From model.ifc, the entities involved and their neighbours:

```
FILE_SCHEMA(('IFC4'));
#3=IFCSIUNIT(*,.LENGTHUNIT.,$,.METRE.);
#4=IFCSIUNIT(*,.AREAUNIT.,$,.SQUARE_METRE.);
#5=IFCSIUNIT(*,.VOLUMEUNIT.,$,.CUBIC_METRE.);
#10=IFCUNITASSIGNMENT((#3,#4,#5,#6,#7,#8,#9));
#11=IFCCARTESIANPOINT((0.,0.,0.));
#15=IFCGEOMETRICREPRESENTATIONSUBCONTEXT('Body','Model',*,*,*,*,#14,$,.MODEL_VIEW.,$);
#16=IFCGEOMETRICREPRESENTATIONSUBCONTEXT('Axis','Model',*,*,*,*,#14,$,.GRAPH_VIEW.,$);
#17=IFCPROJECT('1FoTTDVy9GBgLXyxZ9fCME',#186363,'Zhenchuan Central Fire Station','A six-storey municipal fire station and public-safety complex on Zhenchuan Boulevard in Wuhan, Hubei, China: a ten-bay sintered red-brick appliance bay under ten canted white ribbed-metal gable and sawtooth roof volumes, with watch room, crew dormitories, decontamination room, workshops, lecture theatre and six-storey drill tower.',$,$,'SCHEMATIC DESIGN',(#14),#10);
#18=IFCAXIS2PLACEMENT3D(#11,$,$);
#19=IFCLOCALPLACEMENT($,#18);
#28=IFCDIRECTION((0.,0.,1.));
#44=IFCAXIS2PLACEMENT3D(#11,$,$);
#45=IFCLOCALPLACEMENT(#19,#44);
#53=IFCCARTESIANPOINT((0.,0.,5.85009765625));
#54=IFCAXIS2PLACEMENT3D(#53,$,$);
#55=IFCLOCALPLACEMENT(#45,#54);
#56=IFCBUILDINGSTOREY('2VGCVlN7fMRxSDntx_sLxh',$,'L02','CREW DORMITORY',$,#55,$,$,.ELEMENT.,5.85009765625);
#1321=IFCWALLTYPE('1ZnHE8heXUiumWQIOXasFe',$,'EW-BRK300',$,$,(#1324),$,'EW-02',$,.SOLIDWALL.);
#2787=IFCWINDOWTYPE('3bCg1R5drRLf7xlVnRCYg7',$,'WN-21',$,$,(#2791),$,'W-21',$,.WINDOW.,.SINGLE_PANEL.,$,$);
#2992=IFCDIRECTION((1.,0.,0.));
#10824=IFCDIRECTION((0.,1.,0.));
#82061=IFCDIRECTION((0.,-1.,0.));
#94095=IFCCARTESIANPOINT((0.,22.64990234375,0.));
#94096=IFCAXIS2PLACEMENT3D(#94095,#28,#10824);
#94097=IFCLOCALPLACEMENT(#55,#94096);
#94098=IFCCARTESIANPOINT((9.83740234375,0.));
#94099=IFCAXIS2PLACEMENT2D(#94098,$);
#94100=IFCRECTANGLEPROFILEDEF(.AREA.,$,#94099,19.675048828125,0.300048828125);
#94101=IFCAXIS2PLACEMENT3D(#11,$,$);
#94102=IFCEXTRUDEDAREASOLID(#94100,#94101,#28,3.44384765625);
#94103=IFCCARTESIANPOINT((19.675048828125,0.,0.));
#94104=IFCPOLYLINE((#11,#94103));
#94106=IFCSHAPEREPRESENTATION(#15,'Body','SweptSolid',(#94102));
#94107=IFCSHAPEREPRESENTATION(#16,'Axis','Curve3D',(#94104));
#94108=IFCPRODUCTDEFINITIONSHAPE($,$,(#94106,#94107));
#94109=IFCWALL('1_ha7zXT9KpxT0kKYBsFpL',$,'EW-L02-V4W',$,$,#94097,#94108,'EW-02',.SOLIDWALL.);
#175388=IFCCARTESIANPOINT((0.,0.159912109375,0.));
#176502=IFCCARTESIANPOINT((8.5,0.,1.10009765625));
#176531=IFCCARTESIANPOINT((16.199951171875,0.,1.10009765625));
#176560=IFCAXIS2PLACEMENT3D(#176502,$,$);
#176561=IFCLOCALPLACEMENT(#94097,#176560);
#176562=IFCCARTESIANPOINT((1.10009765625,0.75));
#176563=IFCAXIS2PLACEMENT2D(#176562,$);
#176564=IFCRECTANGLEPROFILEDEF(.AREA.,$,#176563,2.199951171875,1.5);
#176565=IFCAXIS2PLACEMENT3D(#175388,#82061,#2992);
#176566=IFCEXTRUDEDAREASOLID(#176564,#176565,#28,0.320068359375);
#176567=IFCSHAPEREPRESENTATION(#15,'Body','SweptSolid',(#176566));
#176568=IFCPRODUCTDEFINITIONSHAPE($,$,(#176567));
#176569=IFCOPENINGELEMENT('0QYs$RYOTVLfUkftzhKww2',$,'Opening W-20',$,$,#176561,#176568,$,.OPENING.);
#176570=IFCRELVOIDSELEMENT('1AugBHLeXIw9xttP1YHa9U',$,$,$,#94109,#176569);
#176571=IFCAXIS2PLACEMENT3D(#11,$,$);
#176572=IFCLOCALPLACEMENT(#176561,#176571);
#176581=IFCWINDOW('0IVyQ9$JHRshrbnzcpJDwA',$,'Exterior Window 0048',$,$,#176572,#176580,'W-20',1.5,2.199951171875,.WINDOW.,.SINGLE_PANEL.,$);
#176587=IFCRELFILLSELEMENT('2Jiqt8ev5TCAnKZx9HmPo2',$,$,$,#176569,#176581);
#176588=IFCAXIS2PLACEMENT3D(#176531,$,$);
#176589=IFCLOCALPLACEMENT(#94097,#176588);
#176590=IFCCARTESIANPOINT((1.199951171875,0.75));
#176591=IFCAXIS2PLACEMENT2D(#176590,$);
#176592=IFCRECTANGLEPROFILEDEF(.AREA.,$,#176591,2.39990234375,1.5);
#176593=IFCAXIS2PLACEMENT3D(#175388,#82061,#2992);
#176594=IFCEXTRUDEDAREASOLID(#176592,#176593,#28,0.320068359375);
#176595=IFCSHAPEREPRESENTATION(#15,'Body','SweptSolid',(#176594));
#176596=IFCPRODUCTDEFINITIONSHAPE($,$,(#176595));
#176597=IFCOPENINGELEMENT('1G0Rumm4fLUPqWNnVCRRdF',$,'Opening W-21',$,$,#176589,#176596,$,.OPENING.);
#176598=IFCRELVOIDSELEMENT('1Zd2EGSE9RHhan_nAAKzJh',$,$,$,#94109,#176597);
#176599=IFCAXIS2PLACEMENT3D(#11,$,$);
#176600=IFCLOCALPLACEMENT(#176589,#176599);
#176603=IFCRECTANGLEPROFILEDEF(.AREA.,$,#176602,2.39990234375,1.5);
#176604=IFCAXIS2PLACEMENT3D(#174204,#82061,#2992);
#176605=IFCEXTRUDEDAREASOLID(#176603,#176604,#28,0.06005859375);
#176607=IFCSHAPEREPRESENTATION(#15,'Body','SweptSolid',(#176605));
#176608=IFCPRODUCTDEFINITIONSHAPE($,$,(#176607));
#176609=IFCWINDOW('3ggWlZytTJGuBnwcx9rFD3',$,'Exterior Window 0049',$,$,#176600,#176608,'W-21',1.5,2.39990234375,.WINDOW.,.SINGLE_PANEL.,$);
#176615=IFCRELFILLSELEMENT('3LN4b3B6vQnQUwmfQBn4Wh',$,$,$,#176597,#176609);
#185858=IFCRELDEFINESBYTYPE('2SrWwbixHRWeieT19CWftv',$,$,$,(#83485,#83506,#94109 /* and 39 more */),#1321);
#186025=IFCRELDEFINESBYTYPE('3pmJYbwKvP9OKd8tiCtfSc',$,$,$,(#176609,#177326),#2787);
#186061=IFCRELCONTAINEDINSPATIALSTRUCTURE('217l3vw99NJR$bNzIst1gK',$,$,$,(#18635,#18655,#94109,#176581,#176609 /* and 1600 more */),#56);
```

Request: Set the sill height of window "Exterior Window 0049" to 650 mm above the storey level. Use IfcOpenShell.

```python
import numpy as np
import ifcopenshell
import ifcopenshell.api.geometry
import ifcopenshell.geom
import ifcopenshell.util.element
import ifcopenshell.util.placement
import ifcopenshell.util.shape
import ifcopenshell.util.unit

model = ifcopenshell.open("model.ifc")
unit_scale = ifcopenshell.util.unit.calculate_unit_scale(model)

window = model.by_guid("3ggWlZytTJGuBnwcx9rFD3")
opening = window.FillsVoids[0].RelatingOpeningElement
storey = ifcopenshell.util.element.get_container(window, ifc_class="IfcBuildingStorey")
level = ifcopenshell.util.placement.get_local_placement(storey.ObjectPlacement)[2, 3]

# The opening's origin need not be at the sill, so measure its lowest point.
shape = ifcopenshell.geom.create_shape(ifcopenshell.geom.settings(), opening)
bottom = ifcopenshell.util.shape.get_shape_bottom_elevation(shape, shape.geometry) / unit_scale
dz = level + 0.65 - bottom

shift = np.array([0.0, 0.0, dz])
# The window is placed relative to its opening, so it follows when the opening moves.
matrix = ifcopenshell.util.placement.get_local_placement(opening.ObjectPlacement)
matrix[:3, 3] += shift
ifcopenshell.api.geometry.edit_object_placement(
    model, product=opening, matrix=matrix, is_si=False, should_transform_children=True
)

print(f"moved by {dz * unit_scale:+.3f} m")

model.write("model_edited.ifc")
```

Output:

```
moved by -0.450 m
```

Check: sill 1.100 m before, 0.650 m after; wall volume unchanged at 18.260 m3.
